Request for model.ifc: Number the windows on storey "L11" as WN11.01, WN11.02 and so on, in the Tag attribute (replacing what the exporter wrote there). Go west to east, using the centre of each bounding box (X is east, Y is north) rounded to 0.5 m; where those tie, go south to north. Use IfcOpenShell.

First a look at what the model holds.

```python
import ifcopenshell
import ifcopenshell.util.element
import ifcopenshell.util.placement

model = ifcopenshell.open("model.ifc")
print(model.schema)
storey = next(s for s in model.by_type("IfcBuildingStorey") if s.Name == "L11")
windows = [e for e in ifcopenshell.util.element.get_decomposition(storey) if e.is_a("IfcWindow")]
for e in sorted(windows, key=lambda e: e.id()):
    origin = ifcopenshell.util.placement.get_local_placement(e.ObjectPlacement)[:3, 3]
    print(e.id(), e.Tag, e.Name, origin.round(2) + 0.0, sep=" | ")
```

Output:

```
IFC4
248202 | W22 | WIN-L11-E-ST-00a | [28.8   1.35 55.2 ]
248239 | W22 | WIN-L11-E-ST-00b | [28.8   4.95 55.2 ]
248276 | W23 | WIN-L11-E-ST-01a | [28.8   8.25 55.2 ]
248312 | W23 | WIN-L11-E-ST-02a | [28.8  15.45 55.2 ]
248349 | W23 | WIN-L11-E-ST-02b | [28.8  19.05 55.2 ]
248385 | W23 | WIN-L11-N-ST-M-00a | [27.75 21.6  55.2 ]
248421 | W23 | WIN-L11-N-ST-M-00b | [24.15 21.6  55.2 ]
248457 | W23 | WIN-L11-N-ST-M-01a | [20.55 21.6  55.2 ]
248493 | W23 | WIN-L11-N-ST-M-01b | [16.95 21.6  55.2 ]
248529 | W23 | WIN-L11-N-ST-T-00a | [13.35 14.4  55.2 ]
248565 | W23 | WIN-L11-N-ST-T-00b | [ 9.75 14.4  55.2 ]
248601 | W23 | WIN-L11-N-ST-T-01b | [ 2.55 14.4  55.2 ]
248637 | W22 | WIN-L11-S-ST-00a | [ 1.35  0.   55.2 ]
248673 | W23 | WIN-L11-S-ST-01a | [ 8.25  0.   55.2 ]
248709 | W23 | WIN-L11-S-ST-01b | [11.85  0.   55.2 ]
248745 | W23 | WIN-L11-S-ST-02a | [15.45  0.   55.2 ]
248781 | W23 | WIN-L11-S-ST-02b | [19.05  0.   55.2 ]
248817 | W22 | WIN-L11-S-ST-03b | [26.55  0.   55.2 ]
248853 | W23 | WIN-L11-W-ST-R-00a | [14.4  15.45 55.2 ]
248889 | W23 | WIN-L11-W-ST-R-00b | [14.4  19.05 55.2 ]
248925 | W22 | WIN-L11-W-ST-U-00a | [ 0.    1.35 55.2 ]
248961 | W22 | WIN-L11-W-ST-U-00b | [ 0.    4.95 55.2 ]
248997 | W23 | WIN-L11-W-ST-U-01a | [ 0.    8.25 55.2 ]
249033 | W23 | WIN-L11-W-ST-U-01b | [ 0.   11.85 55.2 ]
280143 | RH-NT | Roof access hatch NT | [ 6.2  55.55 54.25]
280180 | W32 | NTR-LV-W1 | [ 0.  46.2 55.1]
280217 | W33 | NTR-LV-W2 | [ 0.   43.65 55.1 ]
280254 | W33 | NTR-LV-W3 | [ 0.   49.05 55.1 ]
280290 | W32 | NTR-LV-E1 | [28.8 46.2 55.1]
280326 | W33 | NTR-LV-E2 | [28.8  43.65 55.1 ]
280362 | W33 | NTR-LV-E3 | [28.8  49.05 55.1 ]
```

```python
import ifcopenshell
import ifcopenshell.geom
import ifcopenshell.util.element
import ifcopenshell.util.shape

model = ifcopenshell.open("model.ifc")
settings = ifcopenshell.geom.settings()
settings.set("use-world-coords", True)


def centre(element):
    shape = ifcopenshell.geom.create_shape(settings, element)
    return ifcopenshell.util.shape.get_bbox_centroid(shape.geometry)


storey = next(s for s in model.by_type("IfcBuildingStorey") if s.Name == "L11")
windows = [e for e in ifcopenshell.util.element.get_decomposition(storey) if e.is_a("IfcWindow")]

# Insertion points can sit at a corner or the storey origin, so sort by the geometry (in metres).
centres = {e: centre(e) for e in windows}
windows.sort(key=lambda e: (round(centres[e][0] / 0.5), centres[e][1]))

for i, e in enumerate(windows, start=1):
    number = f"WN11.{i:02d}"
    e.Tag = number
    print(e.id(), number)

model.write("model_rev.ifc")
```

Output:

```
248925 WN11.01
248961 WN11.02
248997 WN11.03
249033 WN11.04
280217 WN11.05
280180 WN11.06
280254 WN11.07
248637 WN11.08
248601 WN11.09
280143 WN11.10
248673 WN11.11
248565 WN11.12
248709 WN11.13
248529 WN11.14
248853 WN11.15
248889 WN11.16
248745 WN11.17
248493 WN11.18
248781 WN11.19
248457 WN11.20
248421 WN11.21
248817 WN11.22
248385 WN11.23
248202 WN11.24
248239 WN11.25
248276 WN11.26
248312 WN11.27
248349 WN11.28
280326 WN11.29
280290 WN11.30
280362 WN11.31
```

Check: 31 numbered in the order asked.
